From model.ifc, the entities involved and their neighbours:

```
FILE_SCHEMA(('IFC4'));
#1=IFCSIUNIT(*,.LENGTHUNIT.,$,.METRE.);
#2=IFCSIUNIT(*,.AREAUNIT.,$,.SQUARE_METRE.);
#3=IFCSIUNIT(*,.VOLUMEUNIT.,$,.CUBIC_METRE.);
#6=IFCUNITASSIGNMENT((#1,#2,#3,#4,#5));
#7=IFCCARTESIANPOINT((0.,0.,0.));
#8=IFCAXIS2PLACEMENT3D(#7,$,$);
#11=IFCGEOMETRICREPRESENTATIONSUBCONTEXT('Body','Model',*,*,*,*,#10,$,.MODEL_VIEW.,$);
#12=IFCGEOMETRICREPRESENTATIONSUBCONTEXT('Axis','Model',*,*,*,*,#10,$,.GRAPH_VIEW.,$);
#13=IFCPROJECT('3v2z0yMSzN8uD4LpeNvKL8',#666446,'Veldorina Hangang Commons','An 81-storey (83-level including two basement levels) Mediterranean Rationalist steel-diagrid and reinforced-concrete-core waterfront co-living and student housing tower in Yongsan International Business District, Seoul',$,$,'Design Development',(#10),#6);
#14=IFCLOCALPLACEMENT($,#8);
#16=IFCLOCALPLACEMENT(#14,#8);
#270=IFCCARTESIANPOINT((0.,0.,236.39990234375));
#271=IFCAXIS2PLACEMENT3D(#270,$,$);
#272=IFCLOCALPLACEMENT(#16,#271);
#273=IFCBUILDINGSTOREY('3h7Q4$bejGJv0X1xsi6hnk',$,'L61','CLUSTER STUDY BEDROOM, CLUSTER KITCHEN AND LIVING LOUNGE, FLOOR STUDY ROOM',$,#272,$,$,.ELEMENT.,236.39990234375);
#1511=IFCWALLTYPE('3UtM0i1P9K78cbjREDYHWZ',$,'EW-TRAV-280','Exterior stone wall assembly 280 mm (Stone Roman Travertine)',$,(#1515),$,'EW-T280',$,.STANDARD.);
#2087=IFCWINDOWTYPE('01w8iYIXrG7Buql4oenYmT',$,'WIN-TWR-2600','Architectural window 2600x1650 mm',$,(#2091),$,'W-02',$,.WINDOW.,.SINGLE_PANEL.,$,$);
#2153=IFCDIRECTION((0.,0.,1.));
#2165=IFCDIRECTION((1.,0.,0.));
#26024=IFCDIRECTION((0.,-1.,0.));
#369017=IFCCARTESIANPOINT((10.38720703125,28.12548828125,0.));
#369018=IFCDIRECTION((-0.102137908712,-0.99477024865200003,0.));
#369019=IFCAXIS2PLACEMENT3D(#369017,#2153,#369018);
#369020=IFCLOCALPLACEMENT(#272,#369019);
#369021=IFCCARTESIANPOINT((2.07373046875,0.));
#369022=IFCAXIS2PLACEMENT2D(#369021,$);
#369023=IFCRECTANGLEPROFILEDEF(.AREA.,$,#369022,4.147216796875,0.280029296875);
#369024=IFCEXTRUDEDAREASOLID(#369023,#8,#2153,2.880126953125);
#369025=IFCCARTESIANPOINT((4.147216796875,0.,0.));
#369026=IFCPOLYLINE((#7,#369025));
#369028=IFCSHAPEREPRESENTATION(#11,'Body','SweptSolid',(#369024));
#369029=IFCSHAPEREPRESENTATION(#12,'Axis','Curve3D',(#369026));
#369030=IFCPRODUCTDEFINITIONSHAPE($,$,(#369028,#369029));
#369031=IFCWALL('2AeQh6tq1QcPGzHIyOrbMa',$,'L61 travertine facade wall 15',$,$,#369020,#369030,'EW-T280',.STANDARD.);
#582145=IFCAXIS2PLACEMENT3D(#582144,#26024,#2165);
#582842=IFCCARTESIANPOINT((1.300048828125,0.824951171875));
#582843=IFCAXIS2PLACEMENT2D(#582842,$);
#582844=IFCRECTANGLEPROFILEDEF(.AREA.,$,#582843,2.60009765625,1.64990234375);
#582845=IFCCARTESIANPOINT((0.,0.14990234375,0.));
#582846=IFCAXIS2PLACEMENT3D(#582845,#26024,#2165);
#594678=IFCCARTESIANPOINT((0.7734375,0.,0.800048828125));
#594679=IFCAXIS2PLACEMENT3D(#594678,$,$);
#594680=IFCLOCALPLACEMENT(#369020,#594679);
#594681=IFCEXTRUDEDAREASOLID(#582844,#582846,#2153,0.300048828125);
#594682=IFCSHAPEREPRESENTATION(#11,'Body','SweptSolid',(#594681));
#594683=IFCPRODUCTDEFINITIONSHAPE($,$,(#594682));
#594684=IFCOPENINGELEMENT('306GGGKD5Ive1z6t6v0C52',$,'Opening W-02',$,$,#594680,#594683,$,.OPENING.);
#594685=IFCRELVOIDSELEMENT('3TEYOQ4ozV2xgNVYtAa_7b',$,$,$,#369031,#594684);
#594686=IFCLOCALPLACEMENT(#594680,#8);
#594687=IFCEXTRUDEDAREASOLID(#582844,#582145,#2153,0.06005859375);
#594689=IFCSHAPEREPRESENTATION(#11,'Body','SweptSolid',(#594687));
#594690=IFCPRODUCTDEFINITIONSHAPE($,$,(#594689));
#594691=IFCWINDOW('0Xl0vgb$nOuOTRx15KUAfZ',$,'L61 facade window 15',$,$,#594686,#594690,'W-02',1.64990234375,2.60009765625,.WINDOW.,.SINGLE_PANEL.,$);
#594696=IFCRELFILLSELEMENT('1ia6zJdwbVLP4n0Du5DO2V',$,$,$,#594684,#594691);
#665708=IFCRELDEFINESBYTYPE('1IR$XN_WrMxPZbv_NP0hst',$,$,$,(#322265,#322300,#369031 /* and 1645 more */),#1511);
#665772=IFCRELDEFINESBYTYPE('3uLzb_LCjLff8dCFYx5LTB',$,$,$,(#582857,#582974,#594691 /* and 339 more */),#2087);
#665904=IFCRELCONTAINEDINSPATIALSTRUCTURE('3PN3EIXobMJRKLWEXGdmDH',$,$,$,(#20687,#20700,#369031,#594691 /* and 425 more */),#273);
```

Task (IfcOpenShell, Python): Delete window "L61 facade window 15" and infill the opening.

```python
import ifcopenshell
import ifcopenshell.api.feature
import ifcopenshell.api.root
import ifcopenshell.geom
import ifcopenshell.util.shape

model = ifcopenshell.open("model.ifc")
settings = ifcopenshell.geom.settings()


def volume(element):
    """Net volume in cubic metres, openings subtracted."""
    shape = ifcopenshell.geom.create_shape(settings, element)
    return ifcopenshell.util.shape.get_volume(shape.geometry)


window = model.by_id(594691)
opening = window.FillsVoids[0].RelatingOpeningElement
wall = opening.VoidsElements[0].RelatingBuildingElement
before = volume(wall)

ifcopenshell.api.root.remove_product(model, product=window)
ifcopenshell.api.feature.remove_feature(model, feature=opening)

after = volume(wall)

print(f"wall volume {before:.3f} -> {after:.3f} m3")

model.write("model_updated.ifc")
```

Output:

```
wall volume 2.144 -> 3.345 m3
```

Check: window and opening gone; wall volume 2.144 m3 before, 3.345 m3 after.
